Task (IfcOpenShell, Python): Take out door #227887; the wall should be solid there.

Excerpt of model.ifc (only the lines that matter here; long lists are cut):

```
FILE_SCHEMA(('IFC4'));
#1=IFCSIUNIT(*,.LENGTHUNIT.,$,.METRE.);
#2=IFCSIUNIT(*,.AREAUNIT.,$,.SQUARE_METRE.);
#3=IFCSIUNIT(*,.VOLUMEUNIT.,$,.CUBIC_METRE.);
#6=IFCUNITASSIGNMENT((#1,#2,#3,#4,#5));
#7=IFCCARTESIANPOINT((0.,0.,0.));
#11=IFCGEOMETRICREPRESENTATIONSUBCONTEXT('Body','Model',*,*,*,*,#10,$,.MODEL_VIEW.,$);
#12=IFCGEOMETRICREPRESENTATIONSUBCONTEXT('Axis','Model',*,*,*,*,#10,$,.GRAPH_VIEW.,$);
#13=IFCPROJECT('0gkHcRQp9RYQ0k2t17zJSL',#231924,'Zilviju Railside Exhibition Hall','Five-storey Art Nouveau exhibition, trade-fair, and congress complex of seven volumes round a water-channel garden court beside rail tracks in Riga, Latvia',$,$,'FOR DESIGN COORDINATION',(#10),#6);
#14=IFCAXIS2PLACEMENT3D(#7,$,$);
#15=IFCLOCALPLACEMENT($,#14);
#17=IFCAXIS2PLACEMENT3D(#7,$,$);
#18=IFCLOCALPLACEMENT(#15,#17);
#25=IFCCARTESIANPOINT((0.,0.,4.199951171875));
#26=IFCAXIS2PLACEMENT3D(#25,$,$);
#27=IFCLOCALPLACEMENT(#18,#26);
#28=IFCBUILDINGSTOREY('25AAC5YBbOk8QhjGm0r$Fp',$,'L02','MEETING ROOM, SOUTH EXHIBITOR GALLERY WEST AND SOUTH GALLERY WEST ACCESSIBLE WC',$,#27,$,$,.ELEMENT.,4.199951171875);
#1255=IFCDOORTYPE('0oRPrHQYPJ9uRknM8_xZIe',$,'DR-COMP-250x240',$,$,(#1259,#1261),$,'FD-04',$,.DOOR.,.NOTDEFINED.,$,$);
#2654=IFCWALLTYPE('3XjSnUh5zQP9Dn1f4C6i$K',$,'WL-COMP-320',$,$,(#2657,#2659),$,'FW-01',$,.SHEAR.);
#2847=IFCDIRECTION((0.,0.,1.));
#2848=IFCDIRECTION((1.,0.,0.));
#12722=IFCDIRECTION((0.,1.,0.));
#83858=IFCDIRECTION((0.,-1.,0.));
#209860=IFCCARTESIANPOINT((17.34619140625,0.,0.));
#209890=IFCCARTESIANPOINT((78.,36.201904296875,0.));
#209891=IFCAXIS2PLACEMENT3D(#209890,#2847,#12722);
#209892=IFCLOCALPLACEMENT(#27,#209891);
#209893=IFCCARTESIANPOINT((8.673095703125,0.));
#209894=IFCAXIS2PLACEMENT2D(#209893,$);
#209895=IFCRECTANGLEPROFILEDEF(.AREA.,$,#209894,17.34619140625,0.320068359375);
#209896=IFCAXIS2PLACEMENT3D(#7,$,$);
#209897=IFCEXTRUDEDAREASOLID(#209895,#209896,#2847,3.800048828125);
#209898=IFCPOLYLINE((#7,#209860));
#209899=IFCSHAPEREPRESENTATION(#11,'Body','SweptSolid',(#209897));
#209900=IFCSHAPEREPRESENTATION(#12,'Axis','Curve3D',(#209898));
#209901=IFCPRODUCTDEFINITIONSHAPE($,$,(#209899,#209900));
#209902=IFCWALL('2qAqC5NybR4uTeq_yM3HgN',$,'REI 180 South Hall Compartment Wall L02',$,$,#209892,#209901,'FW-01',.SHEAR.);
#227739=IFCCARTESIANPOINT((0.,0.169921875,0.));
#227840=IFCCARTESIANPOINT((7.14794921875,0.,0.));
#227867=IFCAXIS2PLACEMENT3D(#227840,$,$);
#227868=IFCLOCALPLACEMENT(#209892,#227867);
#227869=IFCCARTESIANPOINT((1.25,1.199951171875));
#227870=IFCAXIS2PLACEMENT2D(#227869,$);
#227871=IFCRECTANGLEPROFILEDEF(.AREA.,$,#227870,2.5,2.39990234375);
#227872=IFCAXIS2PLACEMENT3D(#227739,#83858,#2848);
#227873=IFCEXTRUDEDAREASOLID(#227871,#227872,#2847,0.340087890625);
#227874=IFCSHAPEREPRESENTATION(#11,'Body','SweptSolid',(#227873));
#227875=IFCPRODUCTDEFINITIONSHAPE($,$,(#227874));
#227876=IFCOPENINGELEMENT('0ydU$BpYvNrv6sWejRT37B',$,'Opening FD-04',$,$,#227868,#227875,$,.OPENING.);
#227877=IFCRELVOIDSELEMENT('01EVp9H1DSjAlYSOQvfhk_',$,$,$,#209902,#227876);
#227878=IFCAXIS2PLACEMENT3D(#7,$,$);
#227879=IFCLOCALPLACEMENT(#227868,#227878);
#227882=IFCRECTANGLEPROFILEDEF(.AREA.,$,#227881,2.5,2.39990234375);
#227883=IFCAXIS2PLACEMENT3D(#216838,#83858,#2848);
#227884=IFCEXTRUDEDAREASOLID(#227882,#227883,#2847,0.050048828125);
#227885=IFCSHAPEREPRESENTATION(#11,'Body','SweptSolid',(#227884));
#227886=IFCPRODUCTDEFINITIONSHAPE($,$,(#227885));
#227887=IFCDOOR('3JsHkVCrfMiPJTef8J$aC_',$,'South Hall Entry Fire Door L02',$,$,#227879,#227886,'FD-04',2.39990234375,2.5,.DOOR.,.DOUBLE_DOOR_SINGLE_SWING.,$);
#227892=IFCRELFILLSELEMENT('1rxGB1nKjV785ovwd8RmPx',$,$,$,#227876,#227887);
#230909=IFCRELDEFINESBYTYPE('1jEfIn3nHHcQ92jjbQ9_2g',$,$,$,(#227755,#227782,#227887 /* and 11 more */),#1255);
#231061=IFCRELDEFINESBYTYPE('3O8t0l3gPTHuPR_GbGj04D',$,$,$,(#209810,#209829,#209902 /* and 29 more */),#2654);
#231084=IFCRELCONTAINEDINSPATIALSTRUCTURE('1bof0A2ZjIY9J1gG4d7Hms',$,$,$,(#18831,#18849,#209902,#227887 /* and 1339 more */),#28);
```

```python
import ifcopenshell
import ifcopenshell.api.feature
import ifcopenshell.api.root
import ifcopenshell.geom
import ifcopenshell.util.shape

model = ifcopenshell.open("model.ifc")
settings = ifcopenshell.geom.settings()


def volume(element):
    """Net volume in cubic metres, openings subtracted."""
    shape = ifcopenshell.geom.create_shape(settings, element)
    return ifcopenshell.util.shape.get_volume(shape.geometry)


door = model.by_guid("3JsHkVCrfMiPJTef8J$aC_")
opening = door.FillsVoids[0].RelatingOpeningElement
wall = opening.VoidsElements[0].RelatingBuildingElement
before = volume(wall)

ifcopenshell.api.root.remove_product(model, product=door)
ifcopenshell.api.feature.remove_feature(model, feature=opening)

after = volume(wall)

print(f"wall volume {before:.3f} -> {after:.3f} m3")

model.write("model_edited.ifc")
```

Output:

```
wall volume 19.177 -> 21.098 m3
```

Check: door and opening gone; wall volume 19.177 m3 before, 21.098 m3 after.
